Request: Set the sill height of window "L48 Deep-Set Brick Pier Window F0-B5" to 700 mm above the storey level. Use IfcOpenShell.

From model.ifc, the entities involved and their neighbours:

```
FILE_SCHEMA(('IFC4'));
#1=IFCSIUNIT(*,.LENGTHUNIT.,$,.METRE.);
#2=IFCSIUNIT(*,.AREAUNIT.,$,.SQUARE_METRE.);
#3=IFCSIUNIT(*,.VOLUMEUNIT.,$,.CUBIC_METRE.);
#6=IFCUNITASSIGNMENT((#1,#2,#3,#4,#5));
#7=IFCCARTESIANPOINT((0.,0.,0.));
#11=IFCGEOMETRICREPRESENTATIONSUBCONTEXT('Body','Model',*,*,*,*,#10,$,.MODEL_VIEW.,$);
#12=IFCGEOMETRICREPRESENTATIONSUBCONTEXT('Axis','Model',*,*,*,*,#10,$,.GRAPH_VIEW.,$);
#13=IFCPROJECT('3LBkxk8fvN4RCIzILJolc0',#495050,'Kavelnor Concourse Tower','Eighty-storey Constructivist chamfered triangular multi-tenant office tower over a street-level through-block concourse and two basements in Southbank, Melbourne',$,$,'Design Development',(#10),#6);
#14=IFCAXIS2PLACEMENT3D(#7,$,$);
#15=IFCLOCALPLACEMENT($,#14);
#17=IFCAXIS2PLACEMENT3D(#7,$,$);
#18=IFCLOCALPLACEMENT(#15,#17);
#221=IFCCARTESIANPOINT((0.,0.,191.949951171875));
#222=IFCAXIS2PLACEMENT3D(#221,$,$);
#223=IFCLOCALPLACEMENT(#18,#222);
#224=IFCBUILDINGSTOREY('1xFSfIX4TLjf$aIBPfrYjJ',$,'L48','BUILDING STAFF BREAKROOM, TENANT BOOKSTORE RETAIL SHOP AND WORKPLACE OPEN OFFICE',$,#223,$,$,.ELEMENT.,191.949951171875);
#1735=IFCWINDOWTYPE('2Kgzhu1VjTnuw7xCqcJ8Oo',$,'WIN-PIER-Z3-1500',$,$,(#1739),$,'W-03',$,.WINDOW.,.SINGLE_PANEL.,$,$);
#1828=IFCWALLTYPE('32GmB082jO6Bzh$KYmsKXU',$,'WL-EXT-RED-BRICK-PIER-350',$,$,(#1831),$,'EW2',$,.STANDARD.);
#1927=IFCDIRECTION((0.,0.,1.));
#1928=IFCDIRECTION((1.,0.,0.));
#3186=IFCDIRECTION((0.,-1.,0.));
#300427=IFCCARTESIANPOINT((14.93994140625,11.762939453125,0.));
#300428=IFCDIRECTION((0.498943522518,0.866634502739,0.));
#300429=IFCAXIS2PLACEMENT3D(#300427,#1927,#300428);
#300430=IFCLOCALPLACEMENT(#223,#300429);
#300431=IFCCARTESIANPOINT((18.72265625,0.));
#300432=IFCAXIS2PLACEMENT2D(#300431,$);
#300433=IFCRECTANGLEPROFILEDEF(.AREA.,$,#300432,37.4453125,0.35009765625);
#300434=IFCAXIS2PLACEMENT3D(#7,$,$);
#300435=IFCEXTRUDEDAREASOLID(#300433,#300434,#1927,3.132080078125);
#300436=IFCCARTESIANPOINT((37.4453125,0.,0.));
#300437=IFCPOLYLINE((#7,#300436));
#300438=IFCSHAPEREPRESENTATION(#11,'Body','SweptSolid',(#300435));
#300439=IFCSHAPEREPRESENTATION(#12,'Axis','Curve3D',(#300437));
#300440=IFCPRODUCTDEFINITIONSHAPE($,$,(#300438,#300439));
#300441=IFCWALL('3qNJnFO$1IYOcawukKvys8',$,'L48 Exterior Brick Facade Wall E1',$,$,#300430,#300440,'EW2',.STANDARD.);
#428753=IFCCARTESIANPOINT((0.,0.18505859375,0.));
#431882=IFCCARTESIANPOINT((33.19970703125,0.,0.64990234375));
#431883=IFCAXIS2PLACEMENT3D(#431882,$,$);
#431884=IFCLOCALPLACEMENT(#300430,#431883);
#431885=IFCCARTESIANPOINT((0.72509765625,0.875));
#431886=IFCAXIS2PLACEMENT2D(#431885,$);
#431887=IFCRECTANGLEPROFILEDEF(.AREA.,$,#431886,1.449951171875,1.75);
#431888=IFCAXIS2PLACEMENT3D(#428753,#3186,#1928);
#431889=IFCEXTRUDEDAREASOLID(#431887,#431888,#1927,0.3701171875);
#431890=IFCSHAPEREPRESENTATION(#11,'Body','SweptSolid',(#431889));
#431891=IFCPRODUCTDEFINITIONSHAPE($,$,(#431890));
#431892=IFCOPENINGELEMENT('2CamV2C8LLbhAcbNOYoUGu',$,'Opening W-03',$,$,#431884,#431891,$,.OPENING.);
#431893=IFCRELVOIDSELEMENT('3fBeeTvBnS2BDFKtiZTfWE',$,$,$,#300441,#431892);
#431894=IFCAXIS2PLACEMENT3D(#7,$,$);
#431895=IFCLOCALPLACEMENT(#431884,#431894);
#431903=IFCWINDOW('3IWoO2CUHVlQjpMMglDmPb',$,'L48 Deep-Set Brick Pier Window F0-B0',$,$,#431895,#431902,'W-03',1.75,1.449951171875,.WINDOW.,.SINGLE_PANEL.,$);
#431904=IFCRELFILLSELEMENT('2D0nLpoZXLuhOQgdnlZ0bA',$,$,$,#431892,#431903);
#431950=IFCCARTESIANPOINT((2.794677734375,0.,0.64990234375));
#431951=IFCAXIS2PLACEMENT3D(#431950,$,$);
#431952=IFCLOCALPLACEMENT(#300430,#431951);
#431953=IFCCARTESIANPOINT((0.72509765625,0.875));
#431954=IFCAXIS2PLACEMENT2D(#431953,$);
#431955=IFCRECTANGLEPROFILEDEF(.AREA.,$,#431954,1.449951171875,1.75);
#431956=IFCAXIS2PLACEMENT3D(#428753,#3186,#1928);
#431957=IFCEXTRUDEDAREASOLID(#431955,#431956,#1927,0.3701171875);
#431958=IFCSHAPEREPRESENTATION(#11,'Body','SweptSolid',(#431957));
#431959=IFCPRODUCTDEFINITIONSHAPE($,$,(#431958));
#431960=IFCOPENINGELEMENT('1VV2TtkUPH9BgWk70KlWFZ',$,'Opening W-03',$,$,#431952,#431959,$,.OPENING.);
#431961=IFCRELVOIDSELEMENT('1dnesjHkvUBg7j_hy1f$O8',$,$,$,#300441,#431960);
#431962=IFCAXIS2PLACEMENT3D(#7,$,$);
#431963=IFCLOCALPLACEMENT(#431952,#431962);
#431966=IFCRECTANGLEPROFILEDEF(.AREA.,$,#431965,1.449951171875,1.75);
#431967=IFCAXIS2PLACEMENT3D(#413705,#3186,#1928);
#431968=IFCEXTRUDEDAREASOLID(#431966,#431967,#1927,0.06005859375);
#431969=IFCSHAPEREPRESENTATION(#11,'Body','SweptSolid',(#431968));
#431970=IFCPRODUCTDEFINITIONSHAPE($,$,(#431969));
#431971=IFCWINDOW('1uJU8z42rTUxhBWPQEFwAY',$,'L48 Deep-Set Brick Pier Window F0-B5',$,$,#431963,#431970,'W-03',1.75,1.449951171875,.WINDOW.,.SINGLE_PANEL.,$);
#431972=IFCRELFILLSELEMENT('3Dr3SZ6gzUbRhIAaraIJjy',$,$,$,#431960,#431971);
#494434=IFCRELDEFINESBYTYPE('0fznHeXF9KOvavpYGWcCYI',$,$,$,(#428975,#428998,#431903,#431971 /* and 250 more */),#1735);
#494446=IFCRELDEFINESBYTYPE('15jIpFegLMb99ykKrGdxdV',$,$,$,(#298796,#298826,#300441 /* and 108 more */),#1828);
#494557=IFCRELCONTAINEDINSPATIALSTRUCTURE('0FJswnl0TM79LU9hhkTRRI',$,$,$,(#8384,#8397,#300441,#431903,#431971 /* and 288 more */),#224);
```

```python
import numpy as np
import ifcopenshell
import ifcopenshell.api.geometry
import ifcopenshell.geom
import ifcopenshell.util.element
import ifcopenshell.util.placement
import ifcopenshell.util.shape
import ifcopenshell.util.unit

model = ifcopenshell.open("model.ifc")
unit_scale = ifcopenshell.util.unit.calculate_unit_scale(model)

window = model.by_guid("1uJU8z42rTUxhBWPQEFwAY")
opening = window.FillsVoids[0].RelatingOpeningElement
storey = ifcopenshell.util.element.get_container(window, ifc_class="IfcBuildingStorey")
level = ifcopenshell.util.placement.get_local_placement(storey.ObjectPlacement)[2, 3]

# The opening's origin need not be at the sill, so measure its lowest point.
shape = ifcopenshell.geom.create_shape(ifcopenshell.geom.settings(), opening)
bottom = ifcopenshell.util.shape.get_shape_bottom_elevation(shape, shape.geometry) / unit_scale
dz = level + 0.7 / unit_scale - bottom

shift = np.array([0.0, 0.0, dz])
# The window is placed relative to its opening, so it follows when the opening moves.
matrix = ifcopenshell.util.placement.get_local_placement(opening.ObjectPlacement)
matrix[:3, 3] += shift
ifcopenshell.api.geometry.edit_object_placement(
    model, product=opening, matrix=matrix, is_si=False, should_transform_children=True
)

print(f"moved by {dz * unit_scale:+.3f} m")

model.write("model_v2.ifc")
```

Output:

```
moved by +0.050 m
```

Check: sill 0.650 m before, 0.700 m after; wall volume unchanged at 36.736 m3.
